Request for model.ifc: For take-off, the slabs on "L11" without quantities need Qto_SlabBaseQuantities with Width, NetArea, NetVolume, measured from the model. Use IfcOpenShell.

First a look at what the model holds.

```python
import ifcopenshell
import ifcopenshell.util.element
import ifcopenshell.util.unit

model = ifcopenshell.open("model.ifc")
print(model.schema)
for unit_type in ("LENGTHUNIT", "AREAUNIT", "VOLUMEUNIT"):
    print(unit_type, ifcopenshell.util.unit.calculate_unit_scale(model, unit_type))
storey = next(s for s in model.by_type("IfcBuildingStorey") if s.Name == "L11")
slabs = [e for e in ifcopenshell.util.element.get_decomposition(storey) if e.is_a("IfcSlab")]
for e in sorted(slabs, key=lambda e: e.id()):
    print(e.id(), e.is_a(), e.Name, list(ifcopenshell.util.element.get_psets(e, qtos_only=True)), sep=" | ")
```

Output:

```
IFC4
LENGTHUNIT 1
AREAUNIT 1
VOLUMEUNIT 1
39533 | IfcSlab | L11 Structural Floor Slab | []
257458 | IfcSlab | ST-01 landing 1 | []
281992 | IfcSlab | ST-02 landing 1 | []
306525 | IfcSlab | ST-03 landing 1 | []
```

```python
import ifcopenshell
import ifcopenshell.api.pset
import ifcopenshell.geom
import ifcopenshell.util.element
import ifcopenshell.util.shape
import ifcopenshell.util.unit

model = ifcopenshell.open("model.ifc")
unit_scale = ifcopenshell.util.unit.calculate_unit_scale(model)
area_scale = ifcopenshell.util.unit.calculate_unit_scale(model, "AREAUNIT")
volume_scale = ifcopenshell.util.unit.calculate_unit_scale(model, "VOLUMEUNIT")
settings = ifcopenshell.geom.settings()

storey = next(s for s in model.by_type("IfcBuildingStorey") if s.Name == "L11")
slabs = [e for e in ifcopenshell.util.element.get_decomposition(storey) if e.is_a("IfcSlab")]

for e in sorted(slabs, key=lambda e: e.id()):
    if ifcopenshell.util.element.get_psets(e, qtos_only=True, should_inherit=False):
        continue
    # Geometry comes back in metres, in the element's own axes.
    shape = ifcopenshell.geom.create_shape(settings, e)
    values = {
        "Width": ifcopenshell.util.shape.get_z(shape.geometry) / unit_scale,
        "NetArea": ifcopenshell.util.shape.get_footprint_area(shape.geometry) / area_scale,
        "NetVolume": ifcopenshell.util.shape.get_volume(shape.geometry) / volume_scale,
    }
    qto = ifcopenshell.api.pset.add_qto(model, product=e, name="Qto_SlabBaseQuantities")
    ifcopenshell.api.pset.edit_qto(model, qto=qto, properties=values)
    print(e.id(), {k: round(v, 3) for k, v in values.items()})

model.write("model_rev.ifc")
```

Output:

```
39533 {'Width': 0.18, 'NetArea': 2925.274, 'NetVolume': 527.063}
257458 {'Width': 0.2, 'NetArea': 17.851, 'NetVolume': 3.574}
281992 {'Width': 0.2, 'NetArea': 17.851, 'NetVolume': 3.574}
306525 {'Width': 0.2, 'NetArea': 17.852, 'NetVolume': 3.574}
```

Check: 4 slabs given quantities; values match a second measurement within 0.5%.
